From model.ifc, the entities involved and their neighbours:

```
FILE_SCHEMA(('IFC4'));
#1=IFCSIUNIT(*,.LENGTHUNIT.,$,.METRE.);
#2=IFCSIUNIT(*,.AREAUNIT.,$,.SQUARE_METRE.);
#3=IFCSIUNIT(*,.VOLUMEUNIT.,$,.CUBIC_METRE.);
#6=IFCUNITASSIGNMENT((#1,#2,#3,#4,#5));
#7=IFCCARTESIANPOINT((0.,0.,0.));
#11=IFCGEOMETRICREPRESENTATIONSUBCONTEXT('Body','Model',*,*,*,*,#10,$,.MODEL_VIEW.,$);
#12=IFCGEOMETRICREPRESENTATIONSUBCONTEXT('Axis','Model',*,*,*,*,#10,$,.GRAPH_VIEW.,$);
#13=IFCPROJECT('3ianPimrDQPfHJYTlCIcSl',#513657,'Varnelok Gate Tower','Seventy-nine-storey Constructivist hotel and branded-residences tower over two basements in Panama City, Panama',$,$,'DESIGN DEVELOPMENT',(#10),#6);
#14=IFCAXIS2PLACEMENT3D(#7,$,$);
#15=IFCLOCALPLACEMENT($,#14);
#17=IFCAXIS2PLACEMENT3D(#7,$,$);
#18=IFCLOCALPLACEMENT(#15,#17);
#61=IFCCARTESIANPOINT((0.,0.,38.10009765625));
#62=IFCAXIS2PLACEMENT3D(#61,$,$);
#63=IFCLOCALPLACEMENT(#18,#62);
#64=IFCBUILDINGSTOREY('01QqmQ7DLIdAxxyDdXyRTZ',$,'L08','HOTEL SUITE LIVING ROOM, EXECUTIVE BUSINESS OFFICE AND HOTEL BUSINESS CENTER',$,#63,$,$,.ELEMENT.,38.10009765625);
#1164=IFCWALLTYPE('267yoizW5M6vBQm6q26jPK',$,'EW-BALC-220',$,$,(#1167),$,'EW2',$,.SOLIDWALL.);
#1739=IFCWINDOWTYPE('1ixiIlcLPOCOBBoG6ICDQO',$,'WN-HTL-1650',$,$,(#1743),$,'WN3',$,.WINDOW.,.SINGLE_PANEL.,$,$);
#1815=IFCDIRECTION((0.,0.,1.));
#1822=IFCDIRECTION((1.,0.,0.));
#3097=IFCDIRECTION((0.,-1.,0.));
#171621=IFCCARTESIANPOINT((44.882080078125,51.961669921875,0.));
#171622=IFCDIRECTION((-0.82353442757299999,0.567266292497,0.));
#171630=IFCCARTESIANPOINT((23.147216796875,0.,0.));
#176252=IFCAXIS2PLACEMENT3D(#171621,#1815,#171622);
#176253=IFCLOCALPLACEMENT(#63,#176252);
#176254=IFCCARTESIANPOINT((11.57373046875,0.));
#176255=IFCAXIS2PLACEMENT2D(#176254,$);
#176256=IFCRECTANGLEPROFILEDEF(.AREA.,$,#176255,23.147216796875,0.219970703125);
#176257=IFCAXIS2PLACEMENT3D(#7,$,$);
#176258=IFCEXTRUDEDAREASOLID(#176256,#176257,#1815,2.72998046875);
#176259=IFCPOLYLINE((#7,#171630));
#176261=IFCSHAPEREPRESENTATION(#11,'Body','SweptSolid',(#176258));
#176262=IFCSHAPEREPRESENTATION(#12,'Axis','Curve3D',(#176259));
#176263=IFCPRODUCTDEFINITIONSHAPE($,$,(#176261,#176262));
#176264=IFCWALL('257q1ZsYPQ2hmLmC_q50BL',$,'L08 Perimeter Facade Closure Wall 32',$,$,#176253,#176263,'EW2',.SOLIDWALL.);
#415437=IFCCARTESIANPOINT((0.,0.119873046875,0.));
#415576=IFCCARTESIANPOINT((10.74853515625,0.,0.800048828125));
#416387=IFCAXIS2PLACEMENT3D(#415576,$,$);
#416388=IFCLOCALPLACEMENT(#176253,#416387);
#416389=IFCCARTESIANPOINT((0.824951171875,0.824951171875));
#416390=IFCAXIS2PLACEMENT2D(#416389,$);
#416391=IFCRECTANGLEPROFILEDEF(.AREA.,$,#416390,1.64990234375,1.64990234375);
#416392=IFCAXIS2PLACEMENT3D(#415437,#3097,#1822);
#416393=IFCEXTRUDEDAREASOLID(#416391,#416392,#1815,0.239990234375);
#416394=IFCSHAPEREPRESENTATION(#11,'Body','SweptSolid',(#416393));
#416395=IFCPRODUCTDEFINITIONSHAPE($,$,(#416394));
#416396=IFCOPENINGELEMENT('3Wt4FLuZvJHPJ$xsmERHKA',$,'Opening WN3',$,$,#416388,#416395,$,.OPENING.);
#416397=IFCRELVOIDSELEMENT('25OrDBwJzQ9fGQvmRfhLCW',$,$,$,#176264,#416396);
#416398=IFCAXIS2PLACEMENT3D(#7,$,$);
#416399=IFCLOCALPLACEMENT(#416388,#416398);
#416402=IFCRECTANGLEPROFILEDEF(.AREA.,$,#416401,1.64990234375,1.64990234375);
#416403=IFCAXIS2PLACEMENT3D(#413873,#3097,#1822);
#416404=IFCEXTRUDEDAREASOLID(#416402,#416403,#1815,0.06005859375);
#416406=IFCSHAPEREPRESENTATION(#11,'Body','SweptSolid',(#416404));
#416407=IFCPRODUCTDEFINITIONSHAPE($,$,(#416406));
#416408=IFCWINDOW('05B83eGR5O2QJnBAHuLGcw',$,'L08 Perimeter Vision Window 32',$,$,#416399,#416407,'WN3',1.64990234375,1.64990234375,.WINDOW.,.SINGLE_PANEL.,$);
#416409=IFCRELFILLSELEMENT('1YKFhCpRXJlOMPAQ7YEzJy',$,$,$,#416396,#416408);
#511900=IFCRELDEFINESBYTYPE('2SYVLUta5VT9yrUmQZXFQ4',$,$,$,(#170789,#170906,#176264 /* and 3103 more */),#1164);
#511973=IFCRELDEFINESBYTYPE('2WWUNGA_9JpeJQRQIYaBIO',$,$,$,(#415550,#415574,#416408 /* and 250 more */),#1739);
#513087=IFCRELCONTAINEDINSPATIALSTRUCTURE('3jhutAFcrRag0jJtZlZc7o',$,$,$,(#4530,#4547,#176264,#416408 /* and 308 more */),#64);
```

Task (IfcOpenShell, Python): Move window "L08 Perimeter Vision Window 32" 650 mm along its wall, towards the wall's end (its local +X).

```python
import ifcopenshell
import ifcopenshell.api.geometry
import ifcopenshell.util.placement
import ifcopenshell.util.unit

model = ifcopenshell.open("model.ifc")
unit_scale = ifcopenshell.util.unit.calculate_unit_scale(model)

window = model.by_guid("05B83eGR5O2QJnBAHuLGcw")
opening = window.FillsVoids[0].RelatingOpeningElement
wall = opening.VoidsElements[0].RelatingBuildingElement

wall_matrix = ifcopenshell.util.placement.get_local_placement(wall.ObjectPlacement)
shift = wall_matrix[:3, 0] * 0.65 / unit_scale
before = ifcopenshell.util.placement.get_local_placement(window.ObjectPlacement)[:3, 3].copy()

# The window is placed relative to its opening, so it follows when the opening moves.
matrix = ifcopenshell.util.placement.get_local_placement(opening.ObjectPlacement)
matrix[:3, 3] += shift
ifcopenshell.api.geometry.edit_object_placement(
    model, product=opening, matrix=matrix, is_si=False, should_transform_children=True
)

after = ifcopenshell.util.placement.get_local_placement(window.ObjectPlacement)[:3, 3]
print("window moved by", (after - before).round(3) + 0.0)

model.write("model_rev.ifc")
```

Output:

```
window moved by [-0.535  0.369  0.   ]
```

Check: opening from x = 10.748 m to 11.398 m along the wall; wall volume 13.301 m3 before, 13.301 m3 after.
